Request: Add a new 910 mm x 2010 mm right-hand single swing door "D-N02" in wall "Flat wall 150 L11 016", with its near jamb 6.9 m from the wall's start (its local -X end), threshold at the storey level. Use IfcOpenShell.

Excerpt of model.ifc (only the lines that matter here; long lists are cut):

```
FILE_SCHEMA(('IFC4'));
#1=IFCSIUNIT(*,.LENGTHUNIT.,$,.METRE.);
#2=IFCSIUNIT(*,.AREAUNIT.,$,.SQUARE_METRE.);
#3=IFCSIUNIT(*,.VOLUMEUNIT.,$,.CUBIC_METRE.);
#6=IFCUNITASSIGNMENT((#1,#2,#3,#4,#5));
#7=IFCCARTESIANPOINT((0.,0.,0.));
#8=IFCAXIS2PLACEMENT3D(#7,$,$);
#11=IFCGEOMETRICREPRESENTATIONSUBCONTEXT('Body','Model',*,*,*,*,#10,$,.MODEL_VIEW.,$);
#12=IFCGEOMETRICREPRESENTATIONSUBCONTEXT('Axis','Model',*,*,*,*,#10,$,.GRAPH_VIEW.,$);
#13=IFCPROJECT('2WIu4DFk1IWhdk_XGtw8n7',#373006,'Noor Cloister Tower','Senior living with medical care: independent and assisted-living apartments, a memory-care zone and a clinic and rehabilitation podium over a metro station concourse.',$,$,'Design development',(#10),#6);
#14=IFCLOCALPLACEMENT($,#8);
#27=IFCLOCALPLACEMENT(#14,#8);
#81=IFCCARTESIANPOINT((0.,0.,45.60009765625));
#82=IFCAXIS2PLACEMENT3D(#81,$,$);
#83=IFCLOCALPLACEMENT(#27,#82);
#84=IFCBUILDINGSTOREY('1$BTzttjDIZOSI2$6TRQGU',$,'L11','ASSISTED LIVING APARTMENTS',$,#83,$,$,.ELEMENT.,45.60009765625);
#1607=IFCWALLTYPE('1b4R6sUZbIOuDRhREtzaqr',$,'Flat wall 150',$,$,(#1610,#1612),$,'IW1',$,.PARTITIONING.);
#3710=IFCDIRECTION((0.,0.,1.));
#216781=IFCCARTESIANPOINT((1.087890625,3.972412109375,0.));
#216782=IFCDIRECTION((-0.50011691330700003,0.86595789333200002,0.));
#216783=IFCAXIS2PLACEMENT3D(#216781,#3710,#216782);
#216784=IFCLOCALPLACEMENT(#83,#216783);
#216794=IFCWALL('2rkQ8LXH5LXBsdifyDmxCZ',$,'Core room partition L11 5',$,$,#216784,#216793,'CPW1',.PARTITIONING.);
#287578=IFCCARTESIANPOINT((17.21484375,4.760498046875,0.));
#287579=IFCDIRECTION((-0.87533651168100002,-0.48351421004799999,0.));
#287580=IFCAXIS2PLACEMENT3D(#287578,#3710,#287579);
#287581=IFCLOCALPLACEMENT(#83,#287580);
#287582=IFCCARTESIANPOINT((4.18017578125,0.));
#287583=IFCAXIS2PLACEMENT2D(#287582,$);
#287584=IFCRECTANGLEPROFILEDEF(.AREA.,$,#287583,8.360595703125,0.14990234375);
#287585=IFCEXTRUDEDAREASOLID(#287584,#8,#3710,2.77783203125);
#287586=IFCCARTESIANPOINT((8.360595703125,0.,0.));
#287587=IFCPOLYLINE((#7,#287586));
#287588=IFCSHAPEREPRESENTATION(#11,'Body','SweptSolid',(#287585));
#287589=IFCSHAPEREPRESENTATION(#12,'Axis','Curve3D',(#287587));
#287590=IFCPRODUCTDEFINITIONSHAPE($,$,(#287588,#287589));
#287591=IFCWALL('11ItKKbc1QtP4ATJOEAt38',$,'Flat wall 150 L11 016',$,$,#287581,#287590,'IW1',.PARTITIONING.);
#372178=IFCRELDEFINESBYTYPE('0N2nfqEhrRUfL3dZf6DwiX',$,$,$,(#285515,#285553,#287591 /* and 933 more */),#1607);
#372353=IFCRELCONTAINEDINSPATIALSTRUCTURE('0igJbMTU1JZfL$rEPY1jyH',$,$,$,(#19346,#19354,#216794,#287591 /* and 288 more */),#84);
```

```python
import numpy as np
import ifcopenshell
import ifcopenshell.api.feature
import ifcopenshell.api.geometry
import ifcopenshell.api.root
import ifcopenshell.api.spatial
import ifcopenshell.geom
import ifcopenshell.util.element
import ifcopenshell.util.placement
import ifcopenshell.util.representation
import ifcopenshell.util.shape
import ifcopenshell.util.unit

model = ifcopenshell.open("model.ifc")
unit_scale = ifcopenshell.util.unit.calculate_unit_scale(model)
settings = ifcopenshell.geom.settings()


def volume(element):
    """Net volume in cubic metres, openings subtracted."""
    shape = ifcopenshell.geom.create_shape(settings, element)
    return ifcopenshell.util.shape.get_volume(shape.geometry)


wall = model.by_id(287591)
storey = ifcopenshell.util.element.get_container(wall, ifc_class="IfcBuildingStorey")
context = ifcopenshell.util.representation.get_context(model, "Model", "Body", "MODEL_VIEW")
before = volume(wall)

width, height, from_end, sill = 0.91, 2.01, 6.9, 0.0  # metres

# The wall runs along its own X axis, and the end named is its -X end.
wall_shape = ifcopenshell.geom.create_shape(settings, wall)
x, y, z = ifcopenshell.util.shape.get_vertices(wall_shape.geometry).T
start = x.min() + from_end
face, thickness = float(y.min()), float(y.max() - y.min())
wall_matrix = ifcopenshell.util.placement.get_local_placement(wall.ObjectPlacement)
level = ifcopenshell.util.placement.get_local_placement(storey.ObjectPlacement)[2, 3]


def in_wall(x, y):
    """Placement at x, y metres in the wall's axes, at sill height."""
    matrix = wall_matrix.copy()
    matrix[:, 3] = wall_matrix @ np.array([x / unit_scale, y / unit_scale, 0.0, 1.0])
    matrix[2, 3] = level + sill / unit_scale
    return matrix


# Opening: a box that overshoots both wall faces by 50 mm.
opening = ifcopenshell.api.root.create_entity(model, ifc_class="IfcOpeningElement", predefined_type="OPENING")
box = ifcopenshell.api.geometry.add_wall_representation(
    model, context=context, length=width, height=height, thickness=thickness + 0.1
)
ifcopenshell.api.geometry.assign_representation(model, product=opening, representation=box)
ifcopenshell.api.geometry.edit_object_placement(model, product=opening, matrix=in_wall(start, face - 0.05), is_si=False)
ifcopenshell.api.feature.add_feature(model, feature=opening, element=wall)

door = ifcopenshell.api.root.create_entity(model, ifc_class="IfcDoor", name="D-N02", predefined_type="DOOR")
door.OverallWidth, door.OverallHeight = width / unit_scale, height / unit_scale
door.OperationType = "SINGLE_SWING_RIGHT"
body = ifcopenshell.api.geometry.add_door_representation(
    model,
    context=context,
    overall_width=door.OverallWidth,
    overall_height=door.OverallHeight,
    operation_type="SINGLE_SWING_RIGHT",
    lining_properties={"LiningDepth": thickness / unit_scale, "ThresholdDepth": thickness / unit_scale},
)
ifcopenshell.api.geometry.assign_representation(model, product=door, representation=body)
ifcopenshell.api.spatial.assign_container(model, products=[door], relating_structure=storey)
ifcopenshell.api.feature.add_filling(model, opening=opening, element=door)

# The lining spans the wall, so the door starts at the wall face.
ifcopenshell.api.geometry.edit_object_placement(model, product=door, matrix=in_wall(start, face), is_si=False)

after = volume(wall)

print(f"wall volume {before:.3f} -> {after:.3f} m3")

model.write("model_edited.ifc")
```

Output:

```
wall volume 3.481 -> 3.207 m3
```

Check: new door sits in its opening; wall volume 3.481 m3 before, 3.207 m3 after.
